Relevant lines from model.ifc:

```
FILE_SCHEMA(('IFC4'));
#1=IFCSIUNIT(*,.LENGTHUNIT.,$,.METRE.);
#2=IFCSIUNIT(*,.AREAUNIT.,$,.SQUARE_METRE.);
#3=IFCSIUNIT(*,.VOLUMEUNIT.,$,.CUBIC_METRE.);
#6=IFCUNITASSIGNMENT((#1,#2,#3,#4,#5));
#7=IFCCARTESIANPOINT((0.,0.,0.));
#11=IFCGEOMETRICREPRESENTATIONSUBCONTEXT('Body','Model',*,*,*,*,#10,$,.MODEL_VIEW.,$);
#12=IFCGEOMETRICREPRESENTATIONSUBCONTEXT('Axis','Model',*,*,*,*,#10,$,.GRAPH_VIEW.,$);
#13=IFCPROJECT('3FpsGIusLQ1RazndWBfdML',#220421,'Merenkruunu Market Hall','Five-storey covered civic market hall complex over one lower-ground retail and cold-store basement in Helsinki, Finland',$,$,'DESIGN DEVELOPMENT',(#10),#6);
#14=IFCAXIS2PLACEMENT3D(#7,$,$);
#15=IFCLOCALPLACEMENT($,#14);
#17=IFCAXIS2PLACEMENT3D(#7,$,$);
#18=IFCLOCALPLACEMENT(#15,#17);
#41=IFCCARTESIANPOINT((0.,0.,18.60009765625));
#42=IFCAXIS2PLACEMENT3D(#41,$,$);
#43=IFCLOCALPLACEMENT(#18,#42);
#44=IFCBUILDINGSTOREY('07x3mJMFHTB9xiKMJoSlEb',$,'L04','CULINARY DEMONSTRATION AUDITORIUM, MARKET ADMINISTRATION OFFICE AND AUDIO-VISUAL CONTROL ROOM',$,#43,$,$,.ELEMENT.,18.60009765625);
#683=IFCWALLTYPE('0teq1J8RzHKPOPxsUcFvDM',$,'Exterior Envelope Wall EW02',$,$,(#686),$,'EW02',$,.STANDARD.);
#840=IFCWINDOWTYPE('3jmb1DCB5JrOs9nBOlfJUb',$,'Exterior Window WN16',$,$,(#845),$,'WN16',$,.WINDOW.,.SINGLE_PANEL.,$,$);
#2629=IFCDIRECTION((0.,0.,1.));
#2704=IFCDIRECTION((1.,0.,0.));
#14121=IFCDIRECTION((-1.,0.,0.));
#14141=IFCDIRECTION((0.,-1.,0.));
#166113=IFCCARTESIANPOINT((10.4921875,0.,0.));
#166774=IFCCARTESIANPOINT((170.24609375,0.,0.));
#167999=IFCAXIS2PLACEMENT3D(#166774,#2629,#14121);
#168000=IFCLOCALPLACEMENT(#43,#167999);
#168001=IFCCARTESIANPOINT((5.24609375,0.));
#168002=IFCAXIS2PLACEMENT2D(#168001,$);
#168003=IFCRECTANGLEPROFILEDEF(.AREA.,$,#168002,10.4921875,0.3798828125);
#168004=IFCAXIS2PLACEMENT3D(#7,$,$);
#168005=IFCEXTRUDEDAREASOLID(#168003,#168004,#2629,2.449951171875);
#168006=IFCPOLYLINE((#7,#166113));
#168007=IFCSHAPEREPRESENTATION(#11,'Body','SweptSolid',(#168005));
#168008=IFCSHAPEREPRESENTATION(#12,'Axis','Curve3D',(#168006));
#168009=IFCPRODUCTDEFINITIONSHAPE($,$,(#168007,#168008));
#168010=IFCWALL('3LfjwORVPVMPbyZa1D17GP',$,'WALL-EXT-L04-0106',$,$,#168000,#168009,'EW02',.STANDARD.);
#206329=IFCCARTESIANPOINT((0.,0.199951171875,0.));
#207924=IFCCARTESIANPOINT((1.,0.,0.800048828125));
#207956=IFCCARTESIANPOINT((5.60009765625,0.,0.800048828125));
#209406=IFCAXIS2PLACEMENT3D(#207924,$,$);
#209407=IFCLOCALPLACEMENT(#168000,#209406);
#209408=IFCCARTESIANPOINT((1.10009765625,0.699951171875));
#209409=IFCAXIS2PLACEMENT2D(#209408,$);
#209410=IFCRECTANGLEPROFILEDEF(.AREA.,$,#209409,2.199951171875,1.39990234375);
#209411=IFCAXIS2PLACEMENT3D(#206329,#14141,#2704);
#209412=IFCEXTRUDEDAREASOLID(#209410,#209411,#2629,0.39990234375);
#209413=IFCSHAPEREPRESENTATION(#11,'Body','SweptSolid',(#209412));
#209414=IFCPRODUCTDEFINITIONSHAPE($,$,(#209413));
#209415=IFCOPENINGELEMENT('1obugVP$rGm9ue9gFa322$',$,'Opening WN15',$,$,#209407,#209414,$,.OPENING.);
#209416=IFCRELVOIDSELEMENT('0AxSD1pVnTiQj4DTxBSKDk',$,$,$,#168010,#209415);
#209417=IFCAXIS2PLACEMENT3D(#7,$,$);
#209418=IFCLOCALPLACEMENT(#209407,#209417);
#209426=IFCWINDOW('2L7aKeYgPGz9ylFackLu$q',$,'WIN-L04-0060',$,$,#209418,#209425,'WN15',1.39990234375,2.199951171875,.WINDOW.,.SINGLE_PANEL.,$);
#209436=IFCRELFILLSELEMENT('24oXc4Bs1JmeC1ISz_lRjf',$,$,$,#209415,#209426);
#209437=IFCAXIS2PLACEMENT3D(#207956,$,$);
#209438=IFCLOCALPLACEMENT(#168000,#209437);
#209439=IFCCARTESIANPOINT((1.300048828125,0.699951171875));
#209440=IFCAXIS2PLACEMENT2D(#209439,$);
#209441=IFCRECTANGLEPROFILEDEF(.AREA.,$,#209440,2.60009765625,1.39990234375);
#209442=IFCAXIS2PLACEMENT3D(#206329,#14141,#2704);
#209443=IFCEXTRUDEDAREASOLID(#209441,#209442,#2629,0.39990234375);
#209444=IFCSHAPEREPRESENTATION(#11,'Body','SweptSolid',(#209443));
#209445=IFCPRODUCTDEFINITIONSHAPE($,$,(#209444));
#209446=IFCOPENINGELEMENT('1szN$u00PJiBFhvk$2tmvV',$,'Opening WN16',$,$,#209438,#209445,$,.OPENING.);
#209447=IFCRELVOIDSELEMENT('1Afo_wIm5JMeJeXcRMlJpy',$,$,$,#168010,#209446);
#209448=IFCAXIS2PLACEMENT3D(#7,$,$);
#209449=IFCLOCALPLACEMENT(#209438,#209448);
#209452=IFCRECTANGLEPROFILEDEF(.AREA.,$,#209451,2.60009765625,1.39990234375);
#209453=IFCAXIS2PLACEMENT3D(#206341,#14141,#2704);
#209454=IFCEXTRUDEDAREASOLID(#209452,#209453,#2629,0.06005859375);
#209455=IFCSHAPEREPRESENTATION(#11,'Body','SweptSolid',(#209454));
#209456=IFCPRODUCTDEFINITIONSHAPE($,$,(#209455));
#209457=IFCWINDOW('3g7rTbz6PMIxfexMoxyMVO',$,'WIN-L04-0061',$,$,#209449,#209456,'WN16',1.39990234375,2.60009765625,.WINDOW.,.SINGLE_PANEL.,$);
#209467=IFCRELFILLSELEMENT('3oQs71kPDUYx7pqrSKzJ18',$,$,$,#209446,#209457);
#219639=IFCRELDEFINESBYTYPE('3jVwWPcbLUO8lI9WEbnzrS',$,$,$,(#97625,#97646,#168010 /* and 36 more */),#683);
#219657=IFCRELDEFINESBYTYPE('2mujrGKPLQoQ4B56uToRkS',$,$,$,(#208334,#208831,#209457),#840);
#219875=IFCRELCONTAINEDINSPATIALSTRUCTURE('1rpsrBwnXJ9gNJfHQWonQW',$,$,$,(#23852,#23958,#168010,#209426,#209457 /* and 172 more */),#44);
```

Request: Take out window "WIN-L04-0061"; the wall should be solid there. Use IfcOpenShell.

```python
import ifcopenshell
import ifcopenshell.api.feature
import ifcopenshell.api.root
import ifcopenshell.geom
import ifcopenshell.util.shape

model = ifcopenshell.open("model.ifc")
settings = ifcopenshell.geom.settings()


def volume(element):
    """Net volume in cubic metres, openings subtracted."""
    shape = ifcopenshell.geom.create_shape(settings, element)
    return ifcopenshell.util.shape.get_volume(shape.geometry)


window = model.by_guid("3g7rTbz6PMIxfexMoxyMVO")
opening = window.FillsVoids[0].RelatingOpeningElement
wall = opening.VoidsElements[0].RelatingBuildingElement
before = volume(wall)

ifcopenshell.api.root.remove_product(model, product=window)
ifcopenshell.api.feature.remove_feature(model, feature=opening)

after = volume(wall)

print(f"wall volume {before:.3f} -> {after:.3f} m3")

model.write("model_updated.ifc")
```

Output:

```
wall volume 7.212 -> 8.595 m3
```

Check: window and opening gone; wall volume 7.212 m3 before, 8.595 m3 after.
